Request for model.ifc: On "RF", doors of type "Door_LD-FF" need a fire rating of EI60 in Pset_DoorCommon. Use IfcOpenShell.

First a look at what the model holds.

```python
import ifcopenshell
import ifcopenshell.util.element

model = ifcopenshell.open("model.ifc")
print(model.schema)
storey = next(s for s in model.by_type("IfcBuildingStorey") if s.Name == "RF")
doors = [e for e in ifcopenshell.util.element.get_decomposition(storey) if e.is_a("IfcDoor")]
seen = {}
for e in doors:
    element_type = ifcopenshell.util.element.get_type(e)
    key = (element_type.Name if element_type != e and element_type else None, ifcopenshell.util.element.get_pset(e, "Pset_DoorCommon", "FireRating"))
    seen[key] = seen.get(key, 0) + 1
for (name, value), count in sorted(seen.items(), key=str):
    print(count, "x", name, "|", value)
```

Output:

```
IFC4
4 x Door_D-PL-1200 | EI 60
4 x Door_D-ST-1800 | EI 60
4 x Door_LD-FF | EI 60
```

```python
import ifcopenshell
import ifcopenshell.api.pset
import ifcopenshell.util.element

model = ifcopenshell.open("model.ifc")

storey = next(s for s in model.by_type("IfcBuildingStorey") if s.Name == "RF")
doors = [e for e in ifcopenshell.util.element.get_decomposition(storey) if e.is_a("IfcDoor")]

count = 0
for e in doors:
    element_type = ifcopenshell.util.element.get_type(e)
    if element_type in (None, e) or element_type.Name != "Door_LD-FF":
        continue
    # add_pset returns the element's existing set when there is one.
    pset = ifcopenshell.api.pset.add_pset(model, product=e, name="Pset_DoorCommon")
    ifcopenshell.api.pset.edit_pset(model, pset=pset, properties={"FireRating": "EI60"})
    count += 1

print(count, "doors updated")

model.write("model-out.ifc")
```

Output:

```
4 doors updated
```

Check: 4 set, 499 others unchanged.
